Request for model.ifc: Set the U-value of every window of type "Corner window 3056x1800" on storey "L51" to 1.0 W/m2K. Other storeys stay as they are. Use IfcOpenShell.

First a look at what the model holds.

```python
import ifcopenshell
import ifcopenshell.util.element

model = ifcopenshell.open("model.ifc")
print(model.schema)
storey = next(s for s in model.by_type("IfcBuildingStorey") if s.Name == "L51")
windows = [e for e in ifcopenshell.util.element.get_decomposition(storey) if e.is_a("IfcWindow")]
seen = {}
for e in windows:
    element_type = ifcopenshell.util.element.get_type(e)
    key = (element_type.Name if element_type != e and element_type else None, ifcopenshell.util.element.get_pset(e, "Pset_WindowCommon", "ThermalTransmittance"))
    seen[key] = seen.get(key, 0) + 1
for (name, value), count in sorted(seen.items(), key=str):
    print(count, "x", name, "|", value)
```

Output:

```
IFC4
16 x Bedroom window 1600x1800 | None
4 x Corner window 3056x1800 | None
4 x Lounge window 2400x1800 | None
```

```python
import ifcopenshell
import ifcopenshell.api.pset
import ifcopenshell.util.element

model = ifcopenshell.open("model.ifc")

storey = next(s for s in model.by_type("IfcBuildingStorey") if s.Name == "L51")
windows = [e for e in ifcopenshell.util.element.get_decomposition(storey) if e.is_a("IfcWindow")]

count = 0
for e in windows:
    element_type = ifcopenshell.util.element.get_type(e)
    if element_type in (None, e) or element_type.Name != "Corner window 3056x1800":
        continue
    found = ifcopenshell.util.element.get_pset(e, "Pset_WindowCommon", should_inherit=False)
    if found:
        pset = model.by_id(found["id"])
        if len(ifcopenshell.util.element.get_elements_by_pset(pset)) > 1:
            pset = ifcopenshell.api.pset.unshare_pset(model, products=[e], pset=pset)[0]
    else:
        pset = ifcopenshell.api.pset.add_pset(model, product=e, name="Pset_WindowCommon")
    ifcopenshell.api.pset.edit_pset(model, pset=pset, properties={"ThermalTransmittance": 1.0})
    count += 1

print(count, "windows updated")

model.write("model_v2.ifc")
```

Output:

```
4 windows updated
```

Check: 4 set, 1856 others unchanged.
